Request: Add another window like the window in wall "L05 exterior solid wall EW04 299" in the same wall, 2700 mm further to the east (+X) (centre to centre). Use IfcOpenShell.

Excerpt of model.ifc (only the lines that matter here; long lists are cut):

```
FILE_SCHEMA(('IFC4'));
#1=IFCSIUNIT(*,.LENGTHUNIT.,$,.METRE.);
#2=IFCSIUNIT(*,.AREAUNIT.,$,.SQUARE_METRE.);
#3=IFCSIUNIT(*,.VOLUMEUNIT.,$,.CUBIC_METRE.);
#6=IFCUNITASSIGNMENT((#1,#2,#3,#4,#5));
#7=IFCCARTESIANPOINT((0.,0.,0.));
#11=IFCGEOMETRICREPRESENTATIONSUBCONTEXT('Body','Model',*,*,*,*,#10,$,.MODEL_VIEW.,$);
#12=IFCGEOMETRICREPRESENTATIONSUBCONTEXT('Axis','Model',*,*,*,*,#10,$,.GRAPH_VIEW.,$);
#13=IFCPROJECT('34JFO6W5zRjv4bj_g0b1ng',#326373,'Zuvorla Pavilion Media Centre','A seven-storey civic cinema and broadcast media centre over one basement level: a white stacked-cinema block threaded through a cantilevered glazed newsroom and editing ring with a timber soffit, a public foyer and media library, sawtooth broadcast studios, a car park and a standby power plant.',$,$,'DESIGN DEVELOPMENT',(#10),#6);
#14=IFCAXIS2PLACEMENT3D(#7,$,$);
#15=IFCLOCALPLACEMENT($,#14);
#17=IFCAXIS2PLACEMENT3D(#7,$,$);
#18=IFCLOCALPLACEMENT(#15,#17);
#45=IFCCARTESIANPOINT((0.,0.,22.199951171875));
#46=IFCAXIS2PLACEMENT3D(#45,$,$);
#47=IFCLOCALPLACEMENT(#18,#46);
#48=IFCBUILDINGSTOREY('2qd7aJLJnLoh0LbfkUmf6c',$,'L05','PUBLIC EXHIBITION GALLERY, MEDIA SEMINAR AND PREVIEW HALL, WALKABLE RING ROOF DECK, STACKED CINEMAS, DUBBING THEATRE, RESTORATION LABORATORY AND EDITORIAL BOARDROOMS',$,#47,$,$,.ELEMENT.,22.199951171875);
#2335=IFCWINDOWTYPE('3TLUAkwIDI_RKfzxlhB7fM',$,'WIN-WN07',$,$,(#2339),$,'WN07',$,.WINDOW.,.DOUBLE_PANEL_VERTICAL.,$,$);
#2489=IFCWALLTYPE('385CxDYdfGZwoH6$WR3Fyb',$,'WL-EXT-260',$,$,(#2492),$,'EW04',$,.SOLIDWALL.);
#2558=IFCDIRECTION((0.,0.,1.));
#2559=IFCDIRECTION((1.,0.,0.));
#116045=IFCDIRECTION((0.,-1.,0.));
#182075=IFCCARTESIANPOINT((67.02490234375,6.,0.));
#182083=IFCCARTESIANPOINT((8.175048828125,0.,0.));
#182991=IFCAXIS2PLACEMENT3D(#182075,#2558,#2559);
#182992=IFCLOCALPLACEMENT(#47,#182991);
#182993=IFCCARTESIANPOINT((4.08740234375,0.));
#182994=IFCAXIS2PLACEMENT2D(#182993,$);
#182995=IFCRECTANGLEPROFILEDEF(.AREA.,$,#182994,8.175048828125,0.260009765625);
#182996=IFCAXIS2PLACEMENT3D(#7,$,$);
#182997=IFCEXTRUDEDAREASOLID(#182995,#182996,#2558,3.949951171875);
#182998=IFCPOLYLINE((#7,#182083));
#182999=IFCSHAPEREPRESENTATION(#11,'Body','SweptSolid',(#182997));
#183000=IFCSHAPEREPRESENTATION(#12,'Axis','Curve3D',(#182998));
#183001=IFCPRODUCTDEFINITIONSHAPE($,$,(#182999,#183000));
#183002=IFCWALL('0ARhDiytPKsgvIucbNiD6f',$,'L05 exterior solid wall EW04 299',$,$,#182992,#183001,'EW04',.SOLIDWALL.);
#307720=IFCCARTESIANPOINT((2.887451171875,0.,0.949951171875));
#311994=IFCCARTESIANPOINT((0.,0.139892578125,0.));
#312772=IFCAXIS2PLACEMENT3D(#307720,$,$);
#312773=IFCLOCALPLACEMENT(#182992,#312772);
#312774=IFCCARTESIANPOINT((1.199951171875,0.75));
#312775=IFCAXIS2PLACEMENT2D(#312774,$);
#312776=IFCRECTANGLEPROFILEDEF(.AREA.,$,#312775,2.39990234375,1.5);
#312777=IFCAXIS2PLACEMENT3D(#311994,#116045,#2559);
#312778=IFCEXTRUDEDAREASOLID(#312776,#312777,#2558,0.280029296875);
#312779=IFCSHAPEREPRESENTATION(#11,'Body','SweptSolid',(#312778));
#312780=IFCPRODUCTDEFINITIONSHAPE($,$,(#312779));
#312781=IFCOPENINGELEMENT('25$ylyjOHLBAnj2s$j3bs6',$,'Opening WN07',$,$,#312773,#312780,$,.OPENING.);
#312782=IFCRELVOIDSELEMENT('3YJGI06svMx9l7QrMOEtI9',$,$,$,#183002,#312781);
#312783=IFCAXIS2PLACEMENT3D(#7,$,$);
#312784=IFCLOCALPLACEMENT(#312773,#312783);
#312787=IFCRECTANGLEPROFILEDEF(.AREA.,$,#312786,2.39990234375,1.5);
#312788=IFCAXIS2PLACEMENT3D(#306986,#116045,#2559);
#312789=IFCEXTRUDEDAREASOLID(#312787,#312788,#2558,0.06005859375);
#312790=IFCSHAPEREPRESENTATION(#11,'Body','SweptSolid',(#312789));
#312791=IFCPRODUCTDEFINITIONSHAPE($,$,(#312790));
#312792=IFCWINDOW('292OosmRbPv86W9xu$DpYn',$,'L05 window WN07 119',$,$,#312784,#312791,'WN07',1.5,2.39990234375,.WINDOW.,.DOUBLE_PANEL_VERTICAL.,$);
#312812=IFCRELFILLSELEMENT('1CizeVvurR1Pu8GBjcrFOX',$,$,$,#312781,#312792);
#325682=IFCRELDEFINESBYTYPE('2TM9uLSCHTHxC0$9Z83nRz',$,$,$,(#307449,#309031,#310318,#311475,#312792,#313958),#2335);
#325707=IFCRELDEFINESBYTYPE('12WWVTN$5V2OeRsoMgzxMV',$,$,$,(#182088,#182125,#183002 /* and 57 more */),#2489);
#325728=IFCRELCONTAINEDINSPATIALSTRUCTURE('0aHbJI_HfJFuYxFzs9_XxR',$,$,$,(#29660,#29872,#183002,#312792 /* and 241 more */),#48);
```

```python
import ifcopenshell
import ifcopenshell.api.feature
import ifcopenshell.api.geometry
import ifcopenshell.api.root
import ifcopenshell.geom
import ifcopenshell.util.element
import ifcopenshell.util.placement
import ifcopenshell.util.shape
import ifcopenshell.util.unit

model = ifcopenshell.open("model.ifc")
unit_scale = ifcopenshell.util.unit.calculate_unit_scale(model)
settings = ifcopenshell.geom.settings()


def volume(element):
    """Net volume in cubic metres, openings subtracted."""
    shape = ifcopenshell.geom.create_shape(settings, element)
    return ifcopenshell.util.shape.get_volume(shape.geometry)


window = model.by_guid("292OosmRbPv86W9xu$DpYn")
opening = window.FillsVoids[0].RelatingOpeningElement
wall = opening.VoidsElements[0].RelatingBuildingElement
before = volume(wall)
shift = ifcopenshell.util.placement.get_local_placement(wall.ObjectPlacement)[:3, 0] * 2.7 / unit_scale

# copy_class copies the void relationship, type, container and properties, but no geometry.
new_opening = ifcopenshell.api.root.copy_class(model, product=opening)
new_opening.Representation = ifcopenshell.util.element.copy_deep(
    model, opening.Representation, exclude=["IfcGeometricRepresentationContext", "IfcRepresentationMap"]
)
new_window = ifcopenshell.api.root.copy_class(model, product=window)
new_window.Representation = ifcopenshell.util.element.copy_deep(
    model, window.Representation, exclude=["IfcGeometricRepresentationContext", "IfcRepresentationMap"]
)
new_window.Tag = None
ifcopenshell.api.feature.add_filling(model, opening=new_opening, element=new_window)

for old, new in ((opening, new_opening), (window, new_window)):
    matrix = ifcopenshell.util.placement.get_local_placement(old.ObjectPlacement)
    matrix[:3, 3] += shift
    ifcopenshell.api.geometry.edit_object_placement(model, product=new, matrix=matrix, is_si=False)

after = volume(wall)

print(f"wall volume {before:.3f} -> {after:.3f} m3")

model.write("model_rev.ifc")
```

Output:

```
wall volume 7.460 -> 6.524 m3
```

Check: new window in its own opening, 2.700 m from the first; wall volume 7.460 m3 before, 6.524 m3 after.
